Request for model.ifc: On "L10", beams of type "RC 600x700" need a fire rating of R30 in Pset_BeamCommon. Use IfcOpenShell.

First a look at what the model holds.

```python
import ifcopenshell
import ifcopenshell.util.element

model = ifcopenshell.open("model.ifc")
print(model.schema)
storey = next(s for s in model.by_type("IfcBuildingStorey") if s.Name == "L10")
beams = [e for e in ifcopenshell.util.element.get_decomposition(storey) if e.is_a("IfcBeam")]
seen = {}
for e in beams:
    element_type = ifcopenshell.util.element.get_type(e)
    key = (element_type.Name if element_type != e and element_type else None, ifcopenshell.util.element.get_pset(e, "Pset_BeamCommon", "FireRating"))
    seen[key] = seen.get(key, 0) + 1
for (name, value), count in sorted(seen.items(), key=str):
    print(count, "x", name, "|", value)
```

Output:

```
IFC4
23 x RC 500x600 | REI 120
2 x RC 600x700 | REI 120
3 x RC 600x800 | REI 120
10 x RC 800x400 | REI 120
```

```python
import ifcopenshell
import ifcopenshell.api.pset
import ifcopenshell.util.element

model = ifcopenshell.open("model.ifc")

storey = next(s for s in model.by_type("IfcBuildingStorey") if s.Name == "L10")
beams = [e for e in ifcopenshell.util.element.get_decomposition(storey) if e.is_a("IfcBeam")]

count = 0
for e in beams:
    element_type = ifcopenshell.util.element.get_type(e)
    if element_type in (None, e) or element_type.Name != "RC 600x700":
        continue
    # add_pset returns the element's existing set when there is one.
    pset = ifcopenshell.api.pset.add_pset(model, product=e, name="Pset_BeamCommon")
    ifcopenshell.api.pset.edit_pset(model, pset=pset, properties={"FireRating": "R30"})
    count += 1

print(count, "beams updated")

model.write("model_updated.ifc")
```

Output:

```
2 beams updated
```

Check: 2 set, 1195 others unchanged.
